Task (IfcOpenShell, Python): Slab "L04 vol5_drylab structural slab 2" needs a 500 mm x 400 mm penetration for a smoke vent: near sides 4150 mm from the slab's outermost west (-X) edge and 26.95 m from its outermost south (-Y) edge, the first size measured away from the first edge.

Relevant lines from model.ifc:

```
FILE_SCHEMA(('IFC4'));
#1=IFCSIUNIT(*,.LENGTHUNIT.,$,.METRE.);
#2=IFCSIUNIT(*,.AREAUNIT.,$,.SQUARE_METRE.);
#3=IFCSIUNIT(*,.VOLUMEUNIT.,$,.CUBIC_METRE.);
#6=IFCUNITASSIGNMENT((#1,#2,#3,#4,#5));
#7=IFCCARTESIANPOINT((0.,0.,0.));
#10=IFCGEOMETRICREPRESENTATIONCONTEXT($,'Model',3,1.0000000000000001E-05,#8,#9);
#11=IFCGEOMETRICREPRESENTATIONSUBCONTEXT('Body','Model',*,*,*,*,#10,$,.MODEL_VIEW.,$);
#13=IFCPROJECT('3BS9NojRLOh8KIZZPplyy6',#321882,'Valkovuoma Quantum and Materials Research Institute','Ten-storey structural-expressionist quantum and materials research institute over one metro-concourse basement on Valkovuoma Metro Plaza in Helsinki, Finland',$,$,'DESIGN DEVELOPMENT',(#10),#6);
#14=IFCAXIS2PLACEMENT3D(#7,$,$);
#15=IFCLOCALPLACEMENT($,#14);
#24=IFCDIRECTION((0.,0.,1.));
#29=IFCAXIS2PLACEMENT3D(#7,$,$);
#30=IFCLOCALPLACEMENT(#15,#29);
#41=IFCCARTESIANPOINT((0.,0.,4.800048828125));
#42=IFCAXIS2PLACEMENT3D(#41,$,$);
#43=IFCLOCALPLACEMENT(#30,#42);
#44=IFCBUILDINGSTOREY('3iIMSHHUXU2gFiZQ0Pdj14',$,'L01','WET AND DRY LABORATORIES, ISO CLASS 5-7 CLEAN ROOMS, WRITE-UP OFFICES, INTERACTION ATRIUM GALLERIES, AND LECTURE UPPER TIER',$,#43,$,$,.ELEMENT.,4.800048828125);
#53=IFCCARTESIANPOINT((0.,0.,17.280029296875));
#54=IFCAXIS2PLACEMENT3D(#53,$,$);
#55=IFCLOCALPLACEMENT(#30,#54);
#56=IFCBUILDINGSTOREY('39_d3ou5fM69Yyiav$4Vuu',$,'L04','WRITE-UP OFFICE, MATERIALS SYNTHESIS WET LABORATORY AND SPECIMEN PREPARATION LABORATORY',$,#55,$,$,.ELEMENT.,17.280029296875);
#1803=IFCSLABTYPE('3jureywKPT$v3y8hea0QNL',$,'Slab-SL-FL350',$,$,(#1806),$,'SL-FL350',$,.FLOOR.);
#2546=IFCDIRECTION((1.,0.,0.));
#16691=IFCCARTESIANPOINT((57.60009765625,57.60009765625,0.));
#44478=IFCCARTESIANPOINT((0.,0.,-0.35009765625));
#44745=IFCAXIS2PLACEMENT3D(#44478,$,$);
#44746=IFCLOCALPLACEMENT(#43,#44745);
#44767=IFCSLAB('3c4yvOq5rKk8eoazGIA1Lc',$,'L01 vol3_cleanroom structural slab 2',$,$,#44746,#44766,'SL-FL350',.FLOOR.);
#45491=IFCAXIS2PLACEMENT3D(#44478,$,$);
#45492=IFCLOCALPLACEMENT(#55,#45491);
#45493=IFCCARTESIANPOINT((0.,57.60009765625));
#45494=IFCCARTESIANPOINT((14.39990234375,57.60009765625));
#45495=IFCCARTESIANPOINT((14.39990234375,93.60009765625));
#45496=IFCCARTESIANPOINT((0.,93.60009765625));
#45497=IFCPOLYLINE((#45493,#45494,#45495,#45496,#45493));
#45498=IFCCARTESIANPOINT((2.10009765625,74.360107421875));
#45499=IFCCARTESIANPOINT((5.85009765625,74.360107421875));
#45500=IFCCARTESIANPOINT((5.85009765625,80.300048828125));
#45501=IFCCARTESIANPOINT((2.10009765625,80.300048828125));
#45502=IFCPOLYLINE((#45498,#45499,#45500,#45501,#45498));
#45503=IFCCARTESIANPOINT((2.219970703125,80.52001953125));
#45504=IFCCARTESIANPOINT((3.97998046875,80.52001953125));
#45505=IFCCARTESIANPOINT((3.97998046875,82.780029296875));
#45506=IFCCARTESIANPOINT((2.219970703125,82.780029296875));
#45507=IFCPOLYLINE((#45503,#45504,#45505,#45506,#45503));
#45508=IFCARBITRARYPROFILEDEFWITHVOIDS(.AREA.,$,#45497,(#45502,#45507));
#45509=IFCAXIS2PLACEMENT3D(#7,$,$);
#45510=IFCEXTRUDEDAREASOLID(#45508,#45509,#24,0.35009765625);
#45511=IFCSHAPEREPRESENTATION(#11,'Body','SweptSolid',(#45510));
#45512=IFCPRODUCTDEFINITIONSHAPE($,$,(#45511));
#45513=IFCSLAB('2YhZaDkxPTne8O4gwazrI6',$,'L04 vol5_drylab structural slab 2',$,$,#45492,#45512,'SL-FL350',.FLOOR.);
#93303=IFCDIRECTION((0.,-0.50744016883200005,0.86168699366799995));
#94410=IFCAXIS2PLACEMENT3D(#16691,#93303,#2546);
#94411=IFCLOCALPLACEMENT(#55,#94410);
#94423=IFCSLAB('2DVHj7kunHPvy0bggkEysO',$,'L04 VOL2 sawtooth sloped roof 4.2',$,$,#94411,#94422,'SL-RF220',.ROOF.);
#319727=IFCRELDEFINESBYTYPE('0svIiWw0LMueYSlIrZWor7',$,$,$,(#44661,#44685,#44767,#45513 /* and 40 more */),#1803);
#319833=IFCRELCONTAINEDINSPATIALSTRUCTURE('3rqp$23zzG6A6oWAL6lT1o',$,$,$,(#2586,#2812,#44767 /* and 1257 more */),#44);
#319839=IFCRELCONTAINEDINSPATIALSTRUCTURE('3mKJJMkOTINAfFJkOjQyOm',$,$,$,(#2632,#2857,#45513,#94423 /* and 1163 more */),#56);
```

```python
import numpy as np
import ifcopenshell
import ifcopenshell.api.feature
import ifcopenshell.api.geometry
import ifcopenshell.api.root
import ifcopenshell.geom
import ifcopenshell.util.placement
import ifcopenshell.util.representation
import ifcopenshell.util.shape
import ifcopenshell.util.unit

model = ifcopenshell.open("model.ifc")
unit_scale = ifcopenshell.util.unit.calculate_unit_scale(model)
settings = ifcopenshell.geom.settings()


def volume(element):
    """Net volume in cubic metres, openings subtracted."""
    shape = ifcopenshell.geom.create_shape(settings, element)
    return ifcopenshell.util.shape.get_volume(shape.geometry)


slab = model.by_guid("2YhZaDkxPTne8O4gwazrI6")
before = volume(slab)

# Extent in the slab's own axes, in metres. The edges named are its -X and -Y sides.
slab_shape = ifcopenshell.geom.create_shape(settings, slab)
vertices = ifcopenshell.util.shape.get_vertices(slab_shape.geometry)
x_min, y_min, bottom = vertices.min(axis=0)
top = vertices[:, 2].max()

opening = ifcopenshell.api.root.create_entity(model, ifc_class="IfcOpeningElement", name="Smoke vent opening", predefined_type="OPENING")
context = ifcopenshell.util.representation.get_context(model, "Model", "Body", "MODEL_VIEW")
width, depth = 0.5, 0.4
outline = [(0.0, 0.0), (width, 0.0), (width, depth), (0.0, depth), (0.0, 0.0)]
# Overshoot both faces by 50 mm so the cut is clean.
shape = ifcopenshell.api.geometry.add_slab_representation(
    model, context=context, depth=top - bottom + 0.1, polyline=outline
)
ifcopenshell.api.geometry.assign_representation(model, product=opening, representation=shape)

matrix = ifcopenshell.util.placement.get_local_placement(slab.ObjectPlacement)
matrix[:, 3] = matrix @ np.append(np.array([x_min + 4.15, y_min + 26.95, bottom - 0.05]) / unit_scale, 1.0)
ifcopenshell.api.geometry.edit_object_placement(model, product=opening, matrix=matrix, is_si=False)
ifcopenshell.api.feature.add_feature(model, feature=opening, element=slab)

after = volume(slab)

print(f"slab volume {before:.3f} -> {after:.3f} m3")

model.write("model_edited.ifc")
```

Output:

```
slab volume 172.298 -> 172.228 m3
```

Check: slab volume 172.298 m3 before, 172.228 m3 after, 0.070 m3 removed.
